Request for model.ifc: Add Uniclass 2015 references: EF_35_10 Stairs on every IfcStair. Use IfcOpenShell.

First a look at what the model holds.

```python
import ifcopenshell

model = ifcopenshell.open("model.ifc")
print(model.schema)
print("classifications:", [c.Name for c in model.by_type("IfcClassification")])
for ifc_class in ("IfcDoor", "IfcRoof", "IfcStair", "IfcWall", "IfcWindow"):
    print(ifc_class, len(model.by_type(ifc_class)))
```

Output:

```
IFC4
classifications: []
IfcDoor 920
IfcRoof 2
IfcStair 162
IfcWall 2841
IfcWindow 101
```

```python
import ifcopenshell
import ifcopenshell.api.classification

model = ifcopenshell.open("model.ifc")

system = ifcopenshell.api.classification.add_classification(model, classification="Uniclass 2015")

codes = {
    "IfcStair": ("EF_35_10", "Stairs"),
}
for ifc_class, (code, name) in codes.items():
    products = model.by_type(ifc_class)
    ifcopenshell.api.classification.add_reference(
        model, products=products, classification=system, identification=code, name=name
    )
    print(code, len(products))

model.write("model_rev.ifc")
```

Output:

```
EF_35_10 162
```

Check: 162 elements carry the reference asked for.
